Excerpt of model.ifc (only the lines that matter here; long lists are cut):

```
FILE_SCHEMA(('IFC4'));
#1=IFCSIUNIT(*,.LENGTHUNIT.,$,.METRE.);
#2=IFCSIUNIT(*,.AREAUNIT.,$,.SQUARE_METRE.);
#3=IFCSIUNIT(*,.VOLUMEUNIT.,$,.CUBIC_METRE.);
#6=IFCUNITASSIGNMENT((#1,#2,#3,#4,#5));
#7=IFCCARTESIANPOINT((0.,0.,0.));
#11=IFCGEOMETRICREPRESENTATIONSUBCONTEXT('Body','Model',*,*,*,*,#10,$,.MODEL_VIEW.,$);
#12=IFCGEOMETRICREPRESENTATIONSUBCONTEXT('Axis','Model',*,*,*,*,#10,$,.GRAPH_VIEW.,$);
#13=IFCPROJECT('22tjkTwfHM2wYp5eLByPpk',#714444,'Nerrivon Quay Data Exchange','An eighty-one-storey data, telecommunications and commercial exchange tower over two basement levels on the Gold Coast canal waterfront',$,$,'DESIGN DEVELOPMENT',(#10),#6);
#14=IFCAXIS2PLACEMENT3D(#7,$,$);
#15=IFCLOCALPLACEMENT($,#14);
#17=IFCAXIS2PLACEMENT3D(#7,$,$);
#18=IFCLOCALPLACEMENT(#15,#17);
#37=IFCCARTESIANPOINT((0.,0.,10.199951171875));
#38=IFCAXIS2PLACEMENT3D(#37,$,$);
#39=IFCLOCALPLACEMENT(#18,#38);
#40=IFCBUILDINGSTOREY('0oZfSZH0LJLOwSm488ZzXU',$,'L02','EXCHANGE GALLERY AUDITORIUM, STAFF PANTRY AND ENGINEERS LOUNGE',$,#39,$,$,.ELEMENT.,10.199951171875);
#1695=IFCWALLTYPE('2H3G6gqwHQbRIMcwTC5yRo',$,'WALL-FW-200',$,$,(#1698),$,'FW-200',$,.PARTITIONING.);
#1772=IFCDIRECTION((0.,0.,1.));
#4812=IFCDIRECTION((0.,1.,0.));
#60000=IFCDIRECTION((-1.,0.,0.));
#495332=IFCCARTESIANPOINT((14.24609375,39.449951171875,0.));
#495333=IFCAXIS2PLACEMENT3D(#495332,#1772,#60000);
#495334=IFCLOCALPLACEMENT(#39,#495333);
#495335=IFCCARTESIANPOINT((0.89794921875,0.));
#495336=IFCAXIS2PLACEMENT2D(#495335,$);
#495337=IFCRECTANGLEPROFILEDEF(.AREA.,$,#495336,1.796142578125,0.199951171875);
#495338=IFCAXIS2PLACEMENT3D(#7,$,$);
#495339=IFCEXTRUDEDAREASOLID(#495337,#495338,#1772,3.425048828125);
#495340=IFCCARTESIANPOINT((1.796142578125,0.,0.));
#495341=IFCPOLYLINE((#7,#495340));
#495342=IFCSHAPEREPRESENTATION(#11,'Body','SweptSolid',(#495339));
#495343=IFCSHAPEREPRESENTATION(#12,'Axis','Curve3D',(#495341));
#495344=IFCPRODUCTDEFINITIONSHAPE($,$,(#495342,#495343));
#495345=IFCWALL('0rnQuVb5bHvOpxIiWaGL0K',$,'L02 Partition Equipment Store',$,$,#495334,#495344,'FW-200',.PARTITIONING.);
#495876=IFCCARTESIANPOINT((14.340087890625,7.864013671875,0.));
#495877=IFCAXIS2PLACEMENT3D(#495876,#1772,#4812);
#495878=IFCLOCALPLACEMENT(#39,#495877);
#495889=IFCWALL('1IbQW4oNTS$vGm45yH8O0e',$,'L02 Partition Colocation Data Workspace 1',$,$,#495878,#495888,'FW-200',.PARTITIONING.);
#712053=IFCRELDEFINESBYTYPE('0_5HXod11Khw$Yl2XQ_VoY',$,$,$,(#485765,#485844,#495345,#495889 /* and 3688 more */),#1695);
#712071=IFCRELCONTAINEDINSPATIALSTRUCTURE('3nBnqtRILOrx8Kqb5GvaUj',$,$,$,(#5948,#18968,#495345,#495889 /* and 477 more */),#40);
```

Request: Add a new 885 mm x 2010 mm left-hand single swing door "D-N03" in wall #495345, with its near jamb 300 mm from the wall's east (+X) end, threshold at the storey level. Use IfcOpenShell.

```python
import numpy as np
import ifcopenshell
import ifcopenshell.api.feature
import ifcopenshell.api.geometry
import ifcopenshell.api.root
import ifcopenshell.api.spatial
import ifcopenshell.geom
import ifcopenshell.util.element
import ifcopenshell.util.placement
import ifcopenshell.util.representation
import ifcopenshell.util.shape
import ifcopenshell.util.unit

model = ifcopenshell.open("model.ifc")
unit_scale = ifcopenshell.util.unit.calculate_unit_scale(model)
settings = ifcopenshell.geom.settings()


def volume(element):
    """Net volume in cubic metres, openings subtracted."""
    shape = ifcopenshell.geom.create_shape(settings, element)
    return ifcopenshell.util.shape.get_volume(shape.geometry)


wall = model.by_guid("0rnQuVb5bHvOpxIiWaGL0K")
storey = ifcopenshell.util.element.get_container(wall, ifc_class="IfcBuildingStorey")
context = ifcopenshell.util.representation.get_context(model, "Model", "Body", "MODEL_VIEW")
before = volume(wall)

width, height, from_end, sill = 0.885, 2.01, 0.3, 0.0  # metres

# The wall runs along its own X axis, and the end named is its -X end.
wall_shape = ifcopenshell.geom.create_shape(settings, wall)
x, y, z = ifcopenshell.util.shape.get_vertices(wall_shape.geometry).T
start = x.min() + from_end
face, thickness = float(y.min()), float(y.max() - y.min())
wall_matrix = ifcopenshell.util.placement.get_local_placement(wall.ObjectPlacement)
level = ifcopenshell.util.placement.get_local_placement(storey.ObjectPlacement)[2, 3]


def in_wall(x, y):
    """Placement at x, y metres in the wall's axes, at sill height."""
    matrix = wall_matrix.copy()
    matrix[:, 3] = wall_matrix @ np.array([x / unit_scale, y / unit_scale, 0.0, 1.0])
    matrix[2, 3] = level + sill / unit_scale
    return matrix


# Opening: a box that overshoots both wall faces by 50 mm.
opening = ifcopenshell.api.root.create_entity(model, ifc_class="IfcOpeningElement", predefined_type="OPENING")
box = ifcopenshell.api.geometry.add_wall_representation(
    model, context=context, length=width, height=height, thickness=thickness + 0.1
)
ifcopenshell.api.geometry.assign_representation(model, product=opening, representation=box)
ifcopenshell.api.geometry.edit_object_placement(model, product=opening, matrix=in_wall(start, face - 0.05), is_si=False)
ifcopenshell.api.feature.add_feature(model, feature=opening, element=wall)

door = ifcopenshell.api.root.create_entity(model, ifc_class="IfcDoor", name="D-N03", predefined_type="DOOR")
door.OverallWidth, door.OverallHeight = width / unit_scale, height / unit_scale
door.OperationType = "SINGLE_SWING_LEFT"
body = ifcopenshell.api.geometry.add_door_representation(
    model,
    context=context,
    overall_width=door.OverallWidth,
    overall_height=door.OverallHeight,
    operation_type="SINGLE_SWING_LEFT",
    lining_properties={"LiningDepth": thickness / unit_scale, "ThresholdDepth": thickness / unit_scale},
)
ifcopenshell.api.geometry.assign_representation(model, product=door, representation=body)
ifcopenshell.api.spatial.assign_container(model, products=[door], relating_structure=storey)
ifcopenshell.api.feature.add_filling(model, opening=opening, element=door)

# The lining spans the wall, so the door starts at the wall face.
ifcopenshell.api.geometry.edit_object_placement(model, product=door, matrix=in_wall(start, face), is_si=False)

after = volume(wall)

print(f"wall volume {before:.3f} -> {after:.3f} m3")

model.write("model_rev.ifc")
```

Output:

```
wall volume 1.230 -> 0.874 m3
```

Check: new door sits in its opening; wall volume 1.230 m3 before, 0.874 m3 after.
